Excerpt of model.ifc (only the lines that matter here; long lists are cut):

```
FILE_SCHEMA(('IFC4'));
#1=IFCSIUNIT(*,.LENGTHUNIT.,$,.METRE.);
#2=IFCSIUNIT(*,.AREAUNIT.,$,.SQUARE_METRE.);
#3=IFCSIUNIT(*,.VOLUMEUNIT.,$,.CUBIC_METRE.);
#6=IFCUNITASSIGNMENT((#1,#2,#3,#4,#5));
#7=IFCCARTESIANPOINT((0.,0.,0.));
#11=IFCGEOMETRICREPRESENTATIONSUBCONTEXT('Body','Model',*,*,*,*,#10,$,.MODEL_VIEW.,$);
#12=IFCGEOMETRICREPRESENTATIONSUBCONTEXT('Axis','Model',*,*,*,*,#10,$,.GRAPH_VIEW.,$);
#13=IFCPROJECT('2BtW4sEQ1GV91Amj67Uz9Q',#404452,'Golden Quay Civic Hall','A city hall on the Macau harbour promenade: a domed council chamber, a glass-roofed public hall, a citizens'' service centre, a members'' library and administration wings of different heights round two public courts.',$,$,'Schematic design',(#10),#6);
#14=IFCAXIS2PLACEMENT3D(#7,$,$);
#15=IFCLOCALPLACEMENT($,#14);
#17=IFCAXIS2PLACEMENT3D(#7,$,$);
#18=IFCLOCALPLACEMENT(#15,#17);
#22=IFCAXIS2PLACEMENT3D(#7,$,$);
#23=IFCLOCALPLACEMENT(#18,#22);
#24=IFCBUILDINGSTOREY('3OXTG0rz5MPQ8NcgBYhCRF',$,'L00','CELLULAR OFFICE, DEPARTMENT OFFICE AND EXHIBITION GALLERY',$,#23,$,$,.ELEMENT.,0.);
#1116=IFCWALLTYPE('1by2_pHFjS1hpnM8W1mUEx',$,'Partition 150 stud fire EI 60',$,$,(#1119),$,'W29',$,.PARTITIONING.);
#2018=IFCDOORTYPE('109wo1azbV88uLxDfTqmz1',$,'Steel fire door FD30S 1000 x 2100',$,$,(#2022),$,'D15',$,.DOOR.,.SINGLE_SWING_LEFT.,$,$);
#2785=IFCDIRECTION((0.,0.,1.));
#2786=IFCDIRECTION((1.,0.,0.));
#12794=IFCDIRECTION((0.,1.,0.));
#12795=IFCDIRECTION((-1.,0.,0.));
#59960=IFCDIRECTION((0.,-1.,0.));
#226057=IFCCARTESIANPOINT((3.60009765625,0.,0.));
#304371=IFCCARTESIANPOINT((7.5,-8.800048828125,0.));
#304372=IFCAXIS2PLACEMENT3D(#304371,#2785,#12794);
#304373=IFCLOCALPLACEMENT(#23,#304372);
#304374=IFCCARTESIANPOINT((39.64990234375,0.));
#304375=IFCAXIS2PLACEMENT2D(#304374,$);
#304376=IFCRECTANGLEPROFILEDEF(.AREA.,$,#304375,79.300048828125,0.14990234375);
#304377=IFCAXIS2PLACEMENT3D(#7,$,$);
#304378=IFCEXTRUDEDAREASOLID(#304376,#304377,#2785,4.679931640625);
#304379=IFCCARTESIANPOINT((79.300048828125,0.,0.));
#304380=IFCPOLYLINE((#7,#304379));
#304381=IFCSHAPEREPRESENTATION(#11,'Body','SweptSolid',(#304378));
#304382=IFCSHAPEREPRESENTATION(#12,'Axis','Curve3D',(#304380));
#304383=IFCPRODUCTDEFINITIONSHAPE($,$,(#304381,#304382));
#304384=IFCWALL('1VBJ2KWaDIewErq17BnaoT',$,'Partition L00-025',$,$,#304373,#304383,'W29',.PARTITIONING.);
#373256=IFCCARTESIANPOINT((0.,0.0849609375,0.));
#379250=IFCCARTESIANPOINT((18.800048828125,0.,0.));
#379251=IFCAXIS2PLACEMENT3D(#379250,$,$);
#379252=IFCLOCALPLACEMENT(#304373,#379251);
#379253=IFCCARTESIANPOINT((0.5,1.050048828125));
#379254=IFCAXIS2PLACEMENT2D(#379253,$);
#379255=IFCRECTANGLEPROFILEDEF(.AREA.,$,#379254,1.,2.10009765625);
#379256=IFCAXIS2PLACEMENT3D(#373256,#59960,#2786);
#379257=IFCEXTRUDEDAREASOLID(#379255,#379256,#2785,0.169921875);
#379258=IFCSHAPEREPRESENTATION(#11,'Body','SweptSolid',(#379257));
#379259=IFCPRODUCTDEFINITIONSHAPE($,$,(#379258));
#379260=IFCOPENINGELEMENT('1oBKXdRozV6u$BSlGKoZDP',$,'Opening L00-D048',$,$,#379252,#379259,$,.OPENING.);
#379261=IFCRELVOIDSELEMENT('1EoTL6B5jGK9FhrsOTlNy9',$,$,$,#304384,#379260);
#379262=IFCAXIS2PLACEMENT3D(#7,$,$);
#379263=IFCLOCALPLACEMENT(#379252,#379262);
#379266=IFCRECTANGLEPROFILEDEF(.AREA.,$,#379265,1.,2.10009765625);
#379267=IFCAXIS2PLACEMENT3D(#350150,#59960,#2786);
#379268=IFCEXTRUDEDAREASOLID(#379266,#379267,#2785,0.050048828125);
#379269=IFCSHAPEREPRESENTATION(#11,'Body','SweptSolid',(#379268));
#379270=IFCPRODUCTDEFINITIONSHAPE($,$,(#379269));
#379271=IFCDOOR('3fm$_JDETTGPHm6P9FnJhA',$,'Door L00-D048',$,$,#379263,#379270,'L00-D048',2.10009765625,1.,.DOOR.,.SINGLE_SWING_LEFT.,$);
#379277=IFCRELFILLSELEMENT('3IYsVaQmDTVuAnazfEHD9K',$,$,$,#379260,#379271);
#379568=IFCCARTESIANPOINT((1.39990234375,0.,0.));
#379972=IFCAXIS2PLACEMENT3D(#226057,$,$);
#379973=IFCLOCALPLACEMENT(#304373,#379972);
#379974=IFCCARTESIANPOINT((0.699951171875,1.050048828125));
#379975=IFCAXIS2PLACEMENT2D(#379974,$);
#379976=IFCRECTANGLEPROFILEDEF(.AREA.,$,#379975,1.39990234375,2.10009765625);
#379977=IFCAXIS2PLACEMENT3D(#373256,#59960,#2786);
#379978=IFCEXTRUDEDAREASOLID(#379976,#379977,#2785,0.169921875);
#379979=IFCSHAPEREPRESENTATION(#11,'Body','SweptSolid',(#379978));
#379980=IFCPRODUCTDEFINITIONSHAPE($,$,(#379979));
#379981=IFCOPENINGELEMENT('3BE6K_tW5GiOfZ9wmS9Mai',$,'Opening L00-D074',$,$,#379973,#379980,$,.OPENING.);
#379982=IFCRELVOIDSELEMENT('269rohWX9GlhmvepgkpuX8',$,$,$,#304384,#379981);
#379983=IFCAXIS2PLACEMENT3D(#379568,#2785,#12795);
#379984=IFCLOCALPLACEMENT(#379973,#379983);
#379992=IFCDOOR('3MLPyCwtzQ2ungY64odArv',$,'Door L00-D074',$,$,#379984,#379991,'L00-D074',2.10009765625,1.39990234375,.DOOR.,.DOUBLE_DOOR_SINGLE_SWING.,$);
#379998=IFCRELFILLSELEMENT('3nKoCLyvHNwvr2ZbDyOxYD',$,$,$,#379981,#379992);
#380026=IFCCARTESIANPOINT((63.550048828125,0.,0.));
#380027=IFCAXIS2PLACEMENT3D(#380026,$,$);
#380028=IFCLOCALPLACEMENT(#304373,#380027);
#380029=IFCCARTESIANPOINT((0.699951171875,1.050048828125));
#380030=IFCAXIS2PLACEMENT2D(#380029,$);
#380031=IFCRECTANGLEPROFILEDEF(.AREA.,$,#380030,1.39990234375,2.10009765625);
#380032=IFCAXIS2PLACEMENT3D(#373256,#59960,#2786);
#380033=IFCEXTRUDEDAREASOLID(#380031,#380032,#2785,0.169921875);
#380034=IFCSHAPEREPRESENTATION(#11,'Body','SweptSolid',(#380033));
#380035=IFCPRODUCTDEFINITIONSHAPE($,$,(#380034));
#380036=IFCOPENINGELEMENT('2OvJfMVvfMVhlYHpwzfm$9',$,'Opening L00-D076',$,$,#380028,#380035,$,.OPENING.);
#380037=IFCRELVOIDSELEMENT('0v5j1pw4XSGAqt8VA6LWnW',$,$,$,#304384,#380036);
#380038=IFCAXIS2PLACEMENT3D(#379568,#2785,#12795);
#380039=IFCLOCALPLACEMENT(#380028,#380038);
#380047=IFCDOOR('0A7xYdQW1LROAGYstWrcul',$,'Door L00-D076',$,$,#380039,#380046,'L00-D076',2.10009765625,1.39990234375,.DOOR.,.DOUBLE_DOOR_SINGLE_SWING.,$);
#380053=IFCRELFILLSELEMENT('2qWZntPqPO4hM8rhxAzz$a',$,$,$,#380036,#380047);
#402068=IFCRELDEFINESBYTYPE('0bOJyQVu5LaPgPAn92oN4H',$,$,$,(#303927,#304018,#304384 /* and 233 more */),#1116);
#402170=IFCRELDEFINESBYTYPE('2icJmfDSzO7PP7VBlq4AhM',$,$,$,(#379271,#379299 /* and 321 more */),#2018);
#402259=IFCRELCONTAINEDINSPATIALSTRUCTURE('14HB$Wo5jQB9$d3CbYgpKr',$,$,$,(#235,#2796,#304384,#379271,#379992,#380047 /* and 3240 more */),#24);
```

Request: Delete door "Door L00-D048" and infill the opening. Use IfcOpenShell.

```python
import ifcopenshell
import ifcopenshell.api.feature
import ifcopenshell.api.root
import ifcopenshell.geom
import ifcopenshell.util.shape

model = ifcopenshell.open("model.ifc")
settings = ifcopenshell.geom.settings()


def volume(element):
    """Net volume in cubic metres, openings subtracted."""
    shape = ifcopenshell.geom.create_shape(settings, element)
    return ifcopenshell.util.shape.get_volume(shape.geometry)


door = model.by_guid("3fm$_JDETTGPHm6P9FnJhA")
opening = door.FillsVoids[0].RelatingOpeningElement
wall = opening.VoidsElements[0].RelatingBuildingElement
before = volume(wall)

ifcopenshell.api.root.remove_product(model, product=door)
ifcopenshell.api.feature.remove_feature(model, feature=opening)

after = volume(wall)

print(f"wall volume {before:.3f} -> {after:.3f} m3")

model.write("model_edited.ifc")
```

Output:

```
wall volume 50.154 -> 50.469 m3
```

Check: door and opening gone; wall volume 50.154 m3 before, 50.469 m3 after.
